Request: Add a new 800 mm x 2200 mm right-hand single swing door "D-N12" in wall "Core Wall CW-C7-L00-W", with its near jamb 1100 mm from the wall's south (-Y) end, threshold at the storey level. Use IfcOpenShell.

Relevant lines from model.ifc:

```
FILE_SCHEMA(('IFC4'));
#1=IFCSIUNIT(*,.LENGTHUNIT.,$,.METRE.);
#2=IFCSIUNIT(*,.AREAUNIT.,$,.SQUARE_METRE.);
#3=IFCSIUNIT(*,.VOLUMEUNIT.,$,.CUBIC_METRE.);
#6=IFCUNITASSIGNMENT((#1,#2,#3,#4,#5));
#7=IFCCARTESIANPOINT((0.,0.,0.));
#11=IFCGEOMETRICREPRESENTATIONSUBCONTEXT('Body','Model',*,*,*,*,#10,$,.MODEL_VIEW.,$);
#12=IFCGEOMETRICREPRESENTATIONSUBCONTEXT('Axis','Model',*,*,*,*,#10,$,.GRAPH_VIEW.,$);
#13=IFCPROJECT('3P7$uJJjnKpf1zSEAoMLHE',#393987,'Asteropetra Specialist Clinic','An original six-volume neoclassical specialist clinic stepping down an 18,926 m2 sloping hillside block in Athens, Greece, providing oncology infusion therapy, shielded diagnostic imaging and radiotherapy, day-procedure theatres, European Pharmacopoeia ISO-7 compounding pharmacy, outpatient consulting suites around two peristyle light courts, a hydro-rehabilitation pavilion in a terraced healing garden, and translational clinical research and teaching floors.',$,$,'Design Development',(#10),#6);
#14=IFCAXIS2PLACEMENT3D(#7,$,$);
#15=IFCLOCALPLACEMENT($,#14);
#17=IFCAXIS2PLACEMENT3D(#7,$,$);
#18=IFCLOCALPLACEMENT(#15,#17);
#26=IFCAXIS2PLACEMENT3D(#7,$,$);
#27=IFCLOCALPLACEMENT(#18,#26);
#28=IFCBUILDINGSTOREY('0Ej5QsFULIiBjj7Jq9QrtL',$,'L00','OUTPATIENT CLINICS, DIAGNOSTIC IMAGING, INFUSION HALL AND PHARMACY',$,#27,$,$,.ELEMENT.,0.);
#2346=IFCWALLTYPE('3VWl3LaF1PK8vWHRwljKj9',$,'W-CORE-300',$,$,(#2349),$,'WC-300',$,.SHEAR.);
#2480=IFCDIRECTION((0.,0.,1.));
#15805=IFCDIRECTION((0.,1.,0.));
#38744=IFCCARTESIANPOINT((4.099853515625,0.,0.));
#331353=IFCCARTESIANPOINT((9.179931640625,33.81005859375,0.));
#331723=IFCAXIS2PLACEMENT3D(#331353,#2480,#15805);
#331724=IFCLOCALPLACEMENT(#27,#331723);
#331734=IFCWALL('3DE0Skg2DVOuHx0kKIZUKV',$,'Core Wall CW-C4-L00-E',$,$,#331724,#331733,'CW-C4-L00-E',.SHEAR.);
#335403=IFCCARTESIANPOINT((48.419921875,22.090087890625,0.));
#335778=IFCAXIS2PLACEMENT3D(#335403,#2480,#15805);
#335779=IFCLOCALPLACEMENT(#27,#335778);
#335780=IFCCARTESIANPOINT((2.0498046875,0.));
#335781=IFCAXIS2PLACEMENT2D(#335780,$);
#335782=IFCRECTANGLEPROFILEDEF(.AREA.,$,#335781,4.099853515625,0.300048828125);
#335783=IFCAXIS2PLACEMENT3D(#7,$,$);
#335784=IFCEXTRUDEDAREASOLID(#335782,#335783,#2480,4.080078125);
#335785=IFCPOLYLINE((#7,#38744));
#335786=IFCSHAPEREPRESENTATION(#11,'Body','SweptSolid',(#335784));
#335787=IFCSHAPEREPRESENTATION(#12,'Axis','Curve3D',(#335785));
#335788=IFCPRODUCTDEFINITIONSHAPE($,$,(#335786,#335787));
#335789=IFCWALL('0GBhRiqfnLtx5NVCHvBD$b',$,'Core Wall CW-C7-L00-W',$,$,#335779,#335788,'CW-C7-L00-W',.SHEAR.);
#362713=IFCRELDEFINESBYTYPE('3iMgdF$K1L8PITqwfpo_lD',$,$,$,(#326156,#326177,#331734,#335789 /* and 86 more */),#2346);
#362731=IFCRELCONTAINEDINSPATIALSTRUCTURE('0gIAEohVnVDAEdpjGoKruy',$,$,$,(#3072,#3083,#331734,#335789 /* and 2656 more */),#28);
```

```python
import numpy as np
import ifcopenshell
import ifcopenshell.api.feature
import ifcopenshell.api.geometry
import ifcopenshell.api.root
import ifcopenshell.api.spatial
import ifcopenshell.geom
import ifcopenshell.util.element
import ifcopenshell.util.placement
import ifcopenshell.util.representation
import ifcopenshell.util.shape
import ifcopenshell.util.unit

model = ifcopenshell.open("model.ifc")
unit_scale = ifcopenshell.util.unit.calculate_unit_scale(model)
settings = ifcopenshell.geom.settings()


def volume(element):
    """Net volume in cubic metres, openings subtracted."""
    shape = ifcopenshell.geom.create_shape(settings, element)
    return ifcopenshell.util.shape.get_volume(shape.geometry)


wall = model.by_guid("0GBhRiqfnLtx5NVCHvBD$b")
storey = ifcopenshell.util.element.get_container(wall, ifc_class="IfcBuildingStorey")
context = ifcopenshell.util.representation.get_context(model, "Model", "Body", "MODEL_VIEW")
before = volume(wall)

width, height, from_end, sill = 0.8, 2.2, 1.1, 0.0  # metres

# The wall runs along its own X axis, and the end named is its -X end.
wall_shape = ifcopenshell.geom.create_shape(settings, wall)
x, y, z = ifcopenshell.util.shape.get_vertices(wall_shape.geometry).T
start = x.min() + from_end
face, thickness = float(y.min()), float(y.max() - y.min())
wall_matrix = ifcopenshell.util.placement.get_local_placement(wall.ObjectPlacement)
level = ifcopenshell.util.placement.get_local_placement(storey.ObjectPlacement)[2, 3]


def in_wall(x, y):
    """Placement at x, y metres in the wall's axes, at sill height."""
    matrix = wall_matrix.copy()
    matrix[:, 3] = wall_matrix @ np.array([x / unit_scale, y / unit_scale, 0.0, 1.0])
    matrix[2, 3] = level + sill / unit_scale
    return matrix


# Opening: a box that overshoots both wall faces by 50 mm.
opening = ifcopenshell.api.root.create_entity(model, ifc_class="IfcOpeningElement", predefined_type="OPENING")
box = ifcopenshell.api.geometry.add_wall_representation(
    model, context=context, length=width, height=height, thickness=thickness + 0.1
)
ifcopenshell.api.geometry.assign_representation(model, product=opening, representation=box)
ifcopenshell.api.geometry.edit_object_placement(model, product=opening, matrix=in_wall(start, face - 0.05), is_si=False)
ifcopenshell.api.feature.add_feature(model, feature=opening, element=wall)

door = ifcopenshell.api.root.create_entity(model, ifc_class="IfcDoor", name="D-N12", predefined_type="DOOR")
door.OverallWidth, door.OverallHeight = width / unit_scale, height / unit_scale
door.OperationType = "SINGLE_SWING_RIGHT"
body = ifcopenshell.api.geometry.add_door_representation(
    model,
    context=context,
    overall_width=door.OverallWidth,
    overall_height=door.OverallHeight,
    operation_type="SINGLE_SWING_RIGHT",
    lining_properties={"LiningDepth": thickness / unit_scale, "ThresholdDepth": thickness / unit_scale},
)
ifcopenshell.api.geometry.assign_representation(model, product=door, representation=body)
ifcopenshell.api.spatial.assign_container(model, products=[door], relating_structure=storey)
ifcopenshell.api.feature.add_filling(model, opening=opening, element=door)

# The lining spans the wall, so the door starts at the wall face.
ifcopenshell.api.geometry.edit_object_placement(model, product=door, matrix=in_wall(start, face), is_si=False)

after = volume(wall)

print(f"wall volume {before:.3f} -> {after:.3f} m3")

model.write("model_v2.ifc")
```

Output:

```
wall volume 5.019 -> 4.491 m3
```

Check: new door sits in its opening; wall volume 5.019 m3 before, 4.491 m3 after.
